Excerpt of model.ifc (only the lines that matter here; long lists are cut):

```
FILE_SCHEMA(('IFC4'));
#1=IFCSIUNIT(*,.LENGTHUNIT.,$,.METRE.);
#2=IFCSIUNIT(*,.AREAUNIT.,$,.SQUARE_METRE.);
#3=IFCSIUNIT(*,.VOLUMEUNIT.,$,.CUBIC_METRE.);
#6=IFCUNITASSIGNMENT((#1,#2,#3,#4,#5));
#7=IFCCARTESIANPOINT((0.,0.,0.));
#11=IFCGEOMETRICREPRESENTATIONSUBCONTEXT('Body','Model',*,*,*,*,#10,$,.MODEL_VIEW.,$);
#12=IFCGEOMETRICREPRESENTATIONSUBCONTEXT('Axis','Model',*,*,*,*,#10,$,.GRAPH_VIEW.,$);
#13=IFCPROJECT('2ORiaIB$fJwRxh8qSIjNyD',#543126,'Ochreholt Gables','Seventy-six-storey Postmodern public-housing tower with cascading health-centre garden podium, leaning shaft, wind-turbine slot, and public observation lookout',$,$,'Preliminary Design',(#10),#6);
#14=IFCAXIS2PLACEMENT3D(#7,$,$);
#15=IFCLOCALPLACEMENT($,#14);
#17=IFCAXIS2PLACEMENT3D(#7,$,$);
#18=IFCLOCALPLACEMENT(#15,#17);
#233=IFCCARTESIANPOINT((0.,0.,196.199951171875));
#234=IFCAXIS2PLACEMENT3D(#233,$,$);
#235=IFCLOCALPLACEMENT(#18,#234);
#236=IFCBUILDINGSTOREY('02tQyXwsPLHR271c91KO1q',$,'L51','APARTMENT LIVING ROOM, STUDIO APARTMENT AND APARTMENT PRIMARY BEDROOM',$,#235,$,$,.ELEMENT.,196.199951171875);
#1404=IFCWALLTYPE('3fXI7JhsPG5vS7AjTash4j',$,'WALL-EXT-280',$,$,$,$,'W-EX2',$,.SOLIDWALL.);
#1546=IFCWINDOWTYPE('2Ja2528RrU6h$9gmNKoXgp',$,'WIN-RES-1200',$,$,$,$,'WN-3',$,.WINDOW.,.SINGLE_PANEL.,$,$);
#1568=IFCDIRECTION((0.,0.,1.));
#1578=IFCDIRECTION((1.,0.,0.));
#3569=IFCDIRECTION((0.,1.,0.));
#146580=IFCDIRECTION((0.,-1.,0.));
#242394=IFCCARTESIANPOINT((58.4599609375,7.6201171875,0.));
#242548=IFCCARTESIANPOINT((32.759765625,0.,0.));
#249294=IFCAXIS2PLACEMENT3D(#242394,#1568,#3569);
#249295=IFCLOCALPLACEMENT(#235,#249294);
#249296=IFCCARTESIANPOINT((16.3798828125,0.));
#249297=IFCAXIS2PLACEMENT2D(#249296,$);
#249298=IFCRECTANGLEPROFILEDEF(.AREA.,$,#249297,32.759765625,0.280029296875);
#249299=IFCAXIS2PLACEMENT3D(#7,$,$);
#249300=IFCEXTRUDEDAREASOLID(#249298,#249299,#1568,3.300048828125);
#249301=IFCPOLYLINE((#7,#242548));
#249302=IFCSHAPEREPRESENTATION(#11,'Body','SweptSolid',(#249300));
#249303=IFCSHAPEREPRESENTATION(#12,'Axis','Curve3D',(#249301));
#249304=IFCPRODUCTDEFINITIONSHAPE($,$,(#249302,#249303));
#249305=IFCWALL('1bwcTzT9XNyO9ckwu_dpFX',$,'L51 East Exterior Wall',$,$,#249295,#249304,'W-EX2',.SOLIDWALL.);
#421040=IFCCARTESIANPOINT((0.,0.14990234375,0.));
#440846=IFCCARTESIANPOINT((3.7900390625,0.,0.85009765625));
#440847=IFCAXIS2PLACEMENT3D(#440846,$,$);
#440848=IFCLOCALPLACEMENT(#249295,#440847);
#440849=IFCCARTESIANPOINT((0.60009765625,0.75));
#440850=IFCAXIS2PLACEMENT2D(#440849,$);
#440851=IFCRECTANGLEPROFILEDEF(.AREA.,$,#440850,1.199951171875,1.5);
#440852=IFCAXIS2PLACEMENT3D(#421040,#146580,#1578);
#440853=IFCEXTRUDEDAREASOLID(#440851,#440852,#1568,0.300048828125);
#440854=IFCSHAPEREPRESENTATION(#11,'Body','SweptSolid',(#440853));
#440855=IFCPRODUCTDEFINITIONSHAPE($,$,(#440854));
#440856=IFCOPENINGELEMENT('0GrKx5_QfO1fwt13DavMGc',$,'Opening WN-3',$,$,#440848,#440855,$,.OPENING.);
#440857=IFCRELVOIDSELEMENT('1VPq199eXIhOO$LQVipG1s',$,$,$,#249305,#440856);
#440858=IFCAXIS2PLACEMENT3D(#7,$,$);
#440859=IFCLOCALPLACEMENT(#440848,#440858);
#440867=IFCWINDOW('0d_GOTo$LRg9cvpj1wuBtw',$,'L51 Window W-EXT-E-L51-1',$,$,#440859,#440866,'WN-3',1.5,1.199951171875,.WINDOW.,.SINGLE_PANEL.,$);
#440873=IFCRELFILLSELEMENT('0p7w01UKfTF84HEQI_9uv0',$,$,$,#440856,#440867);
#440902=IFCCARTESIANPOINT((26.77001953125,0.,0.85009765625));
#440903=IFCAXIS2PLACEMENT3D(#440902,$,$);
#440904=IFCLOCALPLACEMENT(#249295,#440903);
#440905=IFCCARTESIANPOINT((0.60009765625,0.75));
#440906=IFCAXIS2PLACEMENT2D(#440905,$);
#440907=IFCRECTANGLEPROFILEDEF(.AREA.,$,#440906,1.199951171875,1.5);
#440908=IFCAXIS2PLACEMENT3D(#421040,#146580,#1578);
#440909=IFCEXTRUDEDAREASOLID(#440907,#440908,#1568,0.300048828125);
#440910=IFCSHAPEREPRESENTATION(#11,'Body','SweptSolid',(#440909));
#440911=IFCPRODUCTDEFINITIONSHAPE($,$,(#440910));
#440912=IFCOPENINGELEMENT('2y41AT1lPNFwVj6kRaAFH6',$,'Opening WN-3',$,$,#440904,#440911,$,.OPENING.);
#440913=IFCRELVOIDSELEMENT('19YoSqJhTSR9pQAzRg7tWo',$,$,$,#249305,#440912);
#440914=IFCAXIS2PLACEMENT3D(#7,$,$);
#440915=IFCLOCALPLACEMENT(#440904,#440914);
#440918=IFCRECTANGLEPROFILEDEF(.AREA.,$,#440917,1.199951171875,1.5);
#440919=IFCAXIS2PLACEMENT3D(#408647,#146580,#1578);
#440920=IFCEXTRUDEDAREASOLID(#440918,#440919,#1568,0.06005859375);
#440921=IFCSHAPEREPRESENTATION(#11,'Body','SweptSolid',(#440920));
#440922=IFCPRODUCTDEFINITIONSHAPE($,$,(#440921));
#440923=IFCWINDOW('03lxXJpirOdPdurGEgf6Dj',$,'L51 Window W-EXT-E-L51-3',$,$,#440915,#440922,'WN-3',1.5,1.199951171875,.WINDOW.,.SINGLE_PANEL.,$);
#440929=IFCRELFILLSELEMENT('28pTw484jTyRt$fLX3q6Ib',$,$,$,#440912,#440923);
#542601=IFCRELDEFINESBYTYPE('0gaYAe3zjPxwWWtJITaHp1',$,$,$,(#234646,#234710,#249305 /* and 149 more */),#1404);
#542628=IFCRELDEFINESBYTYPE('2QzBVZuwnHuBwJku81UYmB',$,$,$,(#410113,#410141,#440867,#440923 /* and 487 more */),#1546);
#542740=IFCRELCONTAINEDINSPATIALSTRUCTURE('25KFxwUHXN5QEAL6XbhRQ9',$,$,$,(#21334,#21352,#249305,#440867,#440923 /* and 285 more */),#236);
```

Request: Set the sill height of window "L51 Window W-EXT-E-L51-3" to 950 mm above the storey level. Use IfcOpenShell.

```python
import numpy as np
import ifcopenshell
import ifcopenshell.api.geometry
import ifcopenshell.geom
import ifcopenshell.util.element
import ifcopenshell.util.placement
import ifcopenshell.util.shape
import ifcopenshell.util.unit

model = ifcopenshell.open("model.ifc")
unit_scale = ifcopenshell.util.unit.calculate_unit_scale(model)

window = model.by_guid("03lxXJpirOdPdurGEgf6Dj")
opening = window.FillsVoids[0].RelatingOpeningElement
storey = ifcopenshell.util.element.get_container(window, ifc_class="IfcBuildingStorey")
level = ifcopenshell.util.placement.get_local_placement(storey.ObjectPlacement)[2, 3]

# The opening's origin need not be at the sill, so measure its lowest point.
shape = ifcopenshell.geom.create_shape(ifcopenshell.geom.settings(), opening)
bottom = ifcopenshell.util.shape.get_shape_bottom_elevation(shape, shape.geometry) / unit_scale
dz = level + 0.95 - bottom

shift = np.array([0.0, 0.0, dz])
# The window is placed relative to its opening, so it follows when the opening moves.
matrix = ifcopenshell.util.placement.get_local_placement(opening.ObjectPlacement)
matrix[:3, 3] += shift
ifcopenshell.api.geometry.edit_object_placement(
    model, product=opening, matrix=matrix, is_si=False, should_transform_children=True
)

print(f"moved by {dz * unit_scale:+.3f} m")

model.write("model_updated.ifc")
```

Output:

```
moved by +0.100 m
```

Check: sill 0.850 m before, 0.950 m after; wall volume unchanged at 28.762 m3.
